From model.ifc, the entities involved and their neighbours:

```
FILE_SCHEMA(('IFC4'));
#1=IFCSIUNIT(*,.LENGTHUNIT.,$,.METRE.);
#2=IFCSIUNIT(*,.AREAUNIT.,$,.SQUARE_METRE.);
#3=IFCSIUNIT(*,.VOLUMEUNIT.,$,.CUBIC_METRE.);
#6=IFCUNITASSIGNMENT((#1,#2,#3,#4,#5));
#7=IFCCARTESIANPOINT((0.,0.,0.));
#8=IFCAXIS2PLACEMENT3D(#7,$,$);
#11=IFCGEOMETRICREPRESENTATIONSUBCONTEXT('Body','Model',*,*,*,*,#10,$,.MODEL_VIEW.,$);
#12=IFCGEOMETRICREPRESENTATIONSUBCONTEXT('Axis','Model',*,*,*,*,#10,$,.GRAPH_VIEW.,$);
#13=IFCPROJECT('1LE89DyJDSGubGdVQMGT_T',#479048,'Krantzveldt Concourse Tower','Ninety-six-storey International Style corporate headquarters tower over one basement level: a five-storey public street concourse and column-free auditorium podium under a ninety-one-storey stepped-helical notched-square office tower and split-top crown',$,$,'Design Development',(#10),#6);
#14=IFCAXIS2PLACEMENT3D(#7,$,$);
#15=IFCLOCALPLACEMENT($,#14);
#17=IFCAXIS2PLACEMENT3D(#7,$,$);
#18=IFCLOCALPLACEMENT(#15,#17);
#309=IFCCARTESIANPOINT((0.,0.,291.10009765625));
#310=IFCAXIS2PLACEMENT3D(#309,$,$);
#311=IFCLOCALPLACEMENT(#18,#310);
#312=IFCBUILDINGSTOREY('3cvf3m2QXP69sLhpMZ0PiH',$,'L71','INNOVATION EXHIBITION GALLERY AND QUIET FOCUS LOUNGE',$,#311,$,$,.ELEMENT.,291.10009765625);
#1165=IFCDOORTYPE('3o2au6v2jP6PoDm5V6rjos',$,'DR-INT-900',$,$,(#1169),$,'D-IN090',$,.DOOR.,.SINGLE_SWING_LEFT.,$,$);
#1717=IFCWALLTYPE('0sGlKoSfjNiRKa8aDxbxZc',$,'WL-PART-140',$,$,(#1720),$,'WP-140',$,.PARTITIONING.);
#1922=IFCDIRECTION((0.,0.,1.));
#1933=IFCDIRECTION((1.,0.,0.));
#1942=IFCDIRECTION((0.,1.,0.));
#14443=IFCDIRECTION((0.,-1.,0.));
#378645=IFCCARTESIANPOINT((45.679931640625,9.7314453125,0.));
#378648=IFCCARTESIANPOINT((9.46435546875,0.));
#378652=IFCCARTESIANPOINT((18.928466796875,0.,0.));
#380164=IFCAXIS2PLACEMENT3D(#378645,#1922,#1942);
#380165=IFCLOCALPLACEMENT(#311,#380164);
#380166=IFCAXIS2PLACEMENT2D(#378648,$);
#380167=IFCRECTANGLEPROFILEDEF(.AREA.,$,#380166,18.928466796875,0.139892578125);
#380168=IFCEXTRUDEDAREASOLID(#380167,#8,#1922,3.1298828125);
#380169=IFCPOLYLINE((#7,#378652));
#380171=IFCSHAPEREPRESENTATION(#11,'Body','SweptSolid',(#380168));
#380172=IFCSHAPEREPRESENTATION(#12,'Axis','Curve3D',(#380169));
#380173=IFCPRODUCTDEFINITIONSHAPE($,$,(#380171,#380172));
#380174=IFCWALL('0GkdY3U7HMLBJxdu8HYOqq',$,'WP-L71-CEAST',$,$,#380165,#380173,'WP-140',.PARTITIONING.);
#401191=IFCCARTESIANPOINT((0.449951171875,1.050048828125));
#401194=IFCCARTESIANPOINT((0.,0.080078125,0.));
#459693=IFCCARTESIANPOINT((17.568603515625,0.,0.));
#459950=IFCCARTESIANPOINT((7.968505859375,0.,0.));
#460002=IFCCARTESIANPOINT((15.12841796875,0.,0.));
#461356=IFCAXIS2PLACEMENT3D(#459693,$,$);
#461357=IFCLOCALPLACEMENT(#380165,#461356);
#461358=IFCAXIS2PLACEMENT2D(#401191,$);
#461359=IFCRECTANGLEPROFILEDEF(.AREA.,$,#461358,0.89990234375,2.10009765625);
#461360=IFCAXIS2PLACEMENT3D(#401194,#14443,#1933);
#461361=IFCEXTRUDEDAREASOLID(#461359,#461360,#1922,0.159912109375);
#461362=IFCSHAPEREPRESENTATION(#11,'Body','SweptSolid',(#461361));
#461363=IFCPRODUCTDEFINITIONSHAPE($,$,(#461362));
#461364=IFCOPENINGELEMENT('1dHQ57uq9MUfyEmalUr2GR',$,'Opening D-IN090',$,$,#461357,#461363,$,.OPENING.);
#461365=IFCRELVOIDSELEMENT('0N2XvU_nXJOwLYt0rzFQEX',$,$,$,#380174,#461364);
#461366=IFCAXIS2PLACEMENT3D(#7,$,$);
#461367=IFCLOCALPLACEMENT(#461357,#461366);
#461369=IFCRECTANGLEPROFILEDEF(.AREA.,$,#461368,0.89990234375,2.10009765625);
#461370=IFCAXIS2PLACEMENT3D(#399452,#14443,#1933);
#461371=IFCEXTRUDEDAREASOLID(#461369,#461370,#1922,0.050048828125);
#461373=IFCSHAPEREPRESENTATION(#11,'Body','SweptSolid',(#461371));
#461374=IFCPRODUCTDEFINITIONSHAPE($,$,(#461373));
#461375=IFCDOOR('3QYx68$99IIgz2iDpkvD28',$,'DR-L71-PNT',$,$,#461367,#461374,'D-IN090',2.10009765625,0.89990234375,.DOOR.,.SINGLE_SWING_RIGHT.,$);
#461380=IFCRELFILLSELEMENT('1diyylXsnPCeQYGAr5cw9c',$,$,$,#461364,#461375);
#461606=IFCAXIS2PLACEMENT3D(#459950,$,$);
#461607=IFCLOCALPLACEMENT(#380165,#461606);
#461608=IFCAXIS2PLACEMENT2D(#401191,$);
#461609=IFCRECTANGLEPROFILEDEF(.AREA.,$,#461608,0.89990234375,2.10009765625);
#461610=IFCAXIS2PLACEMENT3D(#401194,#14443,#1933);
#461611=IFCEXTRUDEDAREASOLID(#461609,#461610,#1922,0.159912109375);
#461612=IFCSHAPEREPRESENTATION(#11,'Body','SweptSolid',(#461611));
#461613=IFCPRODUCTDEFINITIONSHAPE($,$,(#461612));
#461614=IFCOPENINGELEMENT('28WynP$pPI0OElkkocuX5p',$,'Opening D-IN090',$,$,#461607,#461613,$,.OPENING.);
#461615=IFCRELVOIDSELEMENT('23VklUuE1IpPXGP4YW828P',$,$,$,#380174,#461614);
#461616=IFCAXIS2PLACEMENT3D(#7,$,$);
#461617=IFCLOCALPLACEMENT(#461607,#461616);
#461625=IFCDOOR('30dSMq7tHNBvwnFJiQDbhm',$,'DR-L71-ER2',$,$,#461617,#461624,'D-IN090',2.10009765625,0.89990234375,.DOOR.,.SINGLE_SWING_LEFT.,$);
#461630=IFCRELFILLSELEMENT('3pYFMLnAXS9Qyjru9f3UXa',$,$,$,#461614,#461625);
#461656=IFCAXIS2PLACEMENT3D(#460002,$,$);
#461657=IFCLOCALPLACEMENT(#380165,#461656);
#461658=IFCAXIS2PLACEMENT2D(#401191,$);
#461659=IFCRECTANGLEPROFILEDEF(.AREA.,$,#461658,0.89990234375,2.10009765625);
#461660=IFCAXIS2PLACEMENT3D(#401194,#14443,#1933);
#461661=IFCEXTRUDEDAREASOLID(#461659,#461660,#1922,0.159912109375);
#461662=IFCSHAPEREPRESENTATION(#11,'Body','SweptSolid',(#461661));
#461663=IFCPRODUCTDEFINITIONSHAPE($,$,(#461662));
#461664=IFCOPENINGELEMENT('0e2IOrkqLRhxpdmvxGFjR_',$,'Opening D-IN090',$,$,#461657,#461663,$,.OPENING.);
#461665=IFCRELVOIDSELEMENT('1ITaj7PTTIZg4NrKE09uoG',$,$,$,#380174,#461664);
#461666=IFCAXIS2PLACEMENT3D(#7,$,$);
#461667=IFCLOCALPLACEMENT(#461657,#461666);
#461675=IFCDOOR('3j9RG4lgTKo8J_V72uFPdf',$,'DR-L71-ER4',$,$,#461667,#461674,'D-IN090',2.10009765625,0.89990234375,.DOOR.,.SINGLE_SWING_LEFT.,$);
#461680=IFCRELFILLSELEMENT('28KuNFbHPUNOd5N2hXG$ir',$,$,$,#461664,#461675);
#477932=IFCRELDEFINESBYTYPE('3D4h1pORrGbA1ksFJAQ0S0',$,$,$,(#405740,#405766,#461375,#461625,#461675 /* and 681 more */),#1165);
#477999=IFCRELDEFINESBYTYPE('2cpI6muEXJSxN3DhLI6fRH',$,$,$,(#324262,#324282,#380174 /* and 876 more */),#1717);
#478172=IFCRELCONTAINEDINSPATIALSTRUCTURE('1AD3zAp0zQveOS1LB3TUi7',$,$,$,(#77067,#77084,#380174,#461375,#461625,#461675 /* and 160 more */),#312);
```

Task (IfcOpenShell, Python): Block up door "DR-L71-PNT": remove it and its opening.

```python
import ifcopenshell
import ifcopenshell.api.feature
import ifcopenshell.api.root
import ifcopenshell.geom
import ifcopenshell.util.shape

model = ifcopenshell.open("model.ifc")
settings = ifcopenshell.geom.settings()


def volume(element):
    """Net volume in cubic metres, openings subtracted."""
    shape = ifcopenshell.geom.create_shape(settings, element)
    return ifcopenshell.util.shape.get_volume(shape.geometry)


door = model.by_guid("3QYx68$99IIgz2iDpkvD28")
opening = door.FillsVoids[0].RelatingOpeningElement
wall = opening.VoidsElements[0].RelatingBuildingElement
before = volume(wall)

ifcopenshell.api.root.remove_product(model, product=door)
ifcopenshell.api.feature.remove_feature(model, feature=opening)

after = volume(wall)

print(f"wall volume {before:.3f} -> {after:.3f} m3")

model.write("model_v2.ifc")
```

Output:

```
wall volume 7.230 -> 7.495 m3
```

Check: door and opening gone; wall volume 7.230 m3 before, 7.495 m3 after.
